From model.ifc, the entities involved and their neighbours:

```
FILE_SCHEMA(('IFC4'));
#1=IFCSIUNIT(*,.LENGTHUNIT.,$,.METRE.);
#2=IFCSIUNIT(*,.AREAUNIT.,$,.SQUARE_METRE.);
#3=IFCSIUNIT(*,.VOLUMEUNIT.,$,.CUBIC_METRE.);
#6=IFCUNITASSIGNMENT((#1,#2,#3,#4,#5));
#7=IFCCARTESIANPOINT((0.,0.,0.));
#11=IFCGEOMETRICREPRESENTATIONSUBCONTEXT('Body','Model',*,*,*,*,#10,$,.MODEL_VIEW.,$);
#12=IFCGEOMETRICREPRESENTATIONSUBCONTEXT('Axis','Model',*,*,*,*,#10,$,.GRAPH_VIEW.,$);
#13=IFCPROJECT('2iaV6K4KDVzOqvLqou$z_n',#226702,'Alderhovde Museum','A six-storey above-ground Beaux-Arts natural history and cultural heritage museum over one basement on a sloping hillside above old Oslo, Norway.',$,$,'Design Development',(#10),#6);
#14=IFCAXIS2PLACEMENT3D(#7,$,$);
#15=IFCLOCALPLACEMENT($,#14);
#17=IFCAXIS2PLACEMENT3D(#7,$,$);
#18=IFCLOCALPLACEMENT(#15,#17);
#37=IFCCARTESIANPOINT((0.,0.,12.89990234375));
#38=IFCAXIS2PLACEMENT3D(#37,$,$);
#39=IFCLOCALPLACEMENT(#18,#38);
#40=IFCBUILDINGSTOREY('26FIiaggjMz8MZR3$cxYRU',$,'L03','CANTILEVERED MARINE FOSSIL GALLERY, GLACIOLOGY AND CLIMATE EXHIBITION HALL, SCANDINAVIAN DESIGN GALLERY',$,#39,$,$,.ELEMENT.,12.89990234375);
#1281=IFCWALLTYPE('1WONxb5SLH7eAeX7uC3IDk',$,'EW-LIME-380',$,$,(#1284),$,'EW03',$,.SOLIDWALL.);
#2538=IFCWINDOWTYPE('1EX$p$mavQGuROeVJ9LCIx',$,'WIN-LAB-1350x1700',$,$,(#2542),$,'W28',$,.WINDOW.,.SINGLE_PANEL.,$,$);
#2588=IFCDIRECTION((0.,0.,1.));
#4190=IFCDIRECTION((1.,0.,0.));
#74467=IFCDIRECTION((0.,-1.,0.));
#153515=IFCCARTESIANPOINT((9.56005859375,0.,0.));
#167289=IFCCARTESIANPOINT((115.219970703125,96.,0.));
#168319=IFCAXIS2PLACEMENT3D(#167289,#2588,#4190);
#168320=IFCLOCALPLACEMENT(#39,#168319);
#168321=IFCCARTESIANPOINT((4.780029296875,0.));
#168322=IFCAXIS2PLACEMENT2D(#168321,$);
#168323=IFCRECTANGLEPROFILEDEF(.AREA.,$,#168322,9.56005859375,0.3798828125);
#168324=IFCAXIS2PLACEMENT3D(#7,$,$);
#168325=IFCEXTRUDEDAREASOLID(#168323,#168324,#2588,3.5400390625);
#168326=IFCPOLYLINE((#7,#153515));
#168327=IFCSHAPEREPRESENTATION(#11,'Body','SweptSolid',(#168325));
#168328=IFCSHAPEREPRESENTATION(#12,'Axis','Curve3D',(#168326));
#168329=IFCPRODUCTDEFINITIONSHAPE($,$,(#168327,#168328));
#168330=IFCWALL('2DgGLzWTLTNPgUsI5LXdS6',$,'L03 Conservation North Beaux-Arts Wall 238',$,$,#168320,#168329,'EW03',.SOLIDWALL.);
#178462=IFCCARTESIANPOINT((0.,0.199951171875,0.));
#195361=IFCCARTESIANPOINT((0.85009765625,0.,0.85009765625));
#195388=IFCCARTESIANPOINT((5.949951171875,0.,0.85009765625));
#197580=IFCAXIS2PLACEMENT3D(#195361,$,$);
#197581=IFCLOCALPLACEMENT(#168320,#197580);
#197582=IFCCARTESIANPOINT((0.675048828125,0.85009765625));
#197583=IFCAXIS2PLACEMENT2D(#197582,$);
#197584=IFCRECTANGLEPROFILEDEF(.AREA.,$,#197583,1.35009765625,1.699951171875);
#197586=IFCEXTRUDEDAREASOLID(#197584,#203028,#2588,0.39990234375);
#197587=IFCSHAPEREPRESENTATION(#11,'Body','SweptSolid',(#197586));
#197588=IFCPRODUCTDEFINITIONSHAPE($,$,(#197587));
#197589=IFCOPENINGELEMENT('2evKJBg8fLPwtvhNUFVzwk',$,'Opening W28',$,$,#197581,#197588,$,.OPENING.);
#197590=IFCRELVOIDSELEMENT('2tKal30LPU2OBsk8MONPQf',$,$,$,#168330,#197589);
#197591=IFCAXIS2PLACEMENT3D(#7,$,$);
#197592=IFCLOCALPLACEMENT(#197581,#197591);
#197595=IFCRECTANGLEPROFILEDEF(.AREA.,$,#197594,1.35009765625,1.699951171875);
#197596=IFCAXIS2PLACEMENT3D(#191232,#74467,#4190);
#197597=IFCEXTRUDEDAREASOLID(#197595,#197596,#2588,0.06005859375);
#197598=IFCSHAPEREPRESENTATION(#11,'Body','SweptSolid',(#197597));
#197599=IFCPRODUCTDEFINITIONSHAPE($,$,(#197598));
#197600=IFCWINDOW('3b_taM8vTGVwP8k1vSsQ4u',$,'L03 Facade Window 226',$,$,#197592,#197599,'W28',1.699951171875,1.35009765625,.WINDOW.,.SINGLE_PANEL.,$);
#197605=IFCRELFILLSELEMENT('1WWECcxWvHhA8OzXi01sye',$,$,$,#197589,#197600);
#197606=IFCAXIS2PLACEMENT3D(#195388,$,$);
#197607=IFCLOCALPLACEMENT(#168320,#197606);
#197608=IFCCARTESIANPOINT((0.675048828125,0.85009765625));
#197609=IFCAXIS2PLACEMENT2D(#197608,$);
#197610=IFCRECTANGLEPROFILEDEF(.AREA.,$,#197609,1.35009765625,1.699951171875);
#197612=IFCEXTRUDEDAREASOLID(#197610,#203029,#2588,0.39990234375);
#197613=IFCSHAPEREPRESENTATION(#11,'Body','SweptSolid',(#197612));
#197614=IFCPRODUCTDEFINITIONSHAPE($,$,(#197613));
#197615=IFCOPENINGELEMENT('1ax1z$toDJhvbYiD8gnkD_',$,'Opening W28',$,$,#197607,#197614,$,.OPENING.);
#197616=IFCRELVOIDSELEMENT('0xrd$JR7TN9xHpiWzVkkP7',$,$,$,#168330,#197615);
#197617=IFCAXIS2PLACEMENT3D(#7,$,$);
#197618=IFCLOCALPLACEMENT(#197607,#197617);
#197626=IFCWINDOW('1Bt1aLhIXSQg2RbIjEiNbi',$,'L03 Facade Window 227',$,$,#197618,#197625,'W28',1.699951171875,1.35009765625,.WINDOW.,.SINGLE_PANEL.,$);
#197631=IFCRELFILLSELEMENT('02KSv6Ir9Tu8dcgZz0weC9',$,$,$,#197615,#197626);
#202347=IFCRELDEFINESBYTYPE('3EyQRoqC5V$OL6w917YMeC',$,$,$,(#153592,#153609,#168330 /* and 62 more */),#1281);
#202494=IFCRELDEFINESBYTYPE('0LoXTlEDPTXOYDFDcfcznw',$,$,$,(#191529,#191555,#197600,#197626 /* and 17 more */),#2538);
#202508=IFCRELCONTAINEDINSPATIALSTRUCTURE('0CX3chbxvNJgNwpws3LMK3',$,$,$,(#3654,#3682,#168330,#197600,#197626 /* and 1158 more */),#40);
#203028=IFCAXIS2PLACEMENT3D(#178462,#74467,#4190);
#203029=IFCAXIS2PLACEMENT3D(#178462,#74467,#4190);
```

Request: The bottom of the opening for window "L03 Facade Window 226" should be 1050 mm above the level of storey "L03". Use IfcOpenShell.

```python
import numpy as np
import ifcopenshell
import ifcopenshell.api.geometry
import ifcopenshell.geom
import ifcopenshell.util.element
import ifcopenshell.util.placement
import ifcopenshell.util.shape
import ifcopenshell.util.unit

model = ifcopenshell.open("model.ifc")
unit_scale = ifcopenshell.util.unit.calculate_unit_scale(model)

window = model.by_guid("3b_taM8vTGVwP8k1vSsQ4u")
opening = window.FillsVoids[0].RelatingOpeningElement
storey = ifcopenshell.util.element.get_container(window, ifc_class="IfcBuildingStorey")
level = ifcopenshell.util.placement.get_local_placement(storey.ObjectPlacement)[2, 3]

# The opening's origin need not be at the sill, so measure its lowest point.
shape = ifcopenshell.geom.create_shape(ifcopenshell.geom.settings(), opening)
bottom = ifcopenshell.util.shape.get_shape_bottom_elevation(shape, shape.geometry) / unit_scale
dz = level + 1.05 / unit_scale - bottom

shift = np.array([0.0, 0.0, dz])
# The window is placed relative to its opening, so it follows when the opening moves.
matrix = ifcopenshell.util.placement.get_local_placement(opening.ObjectPlacement)
matrix[:3, 3] += shift
ifcopenshell.api.geometry.edit_object_placement(
    model, product=opening, matrix=matrix, is_si=False, should_transform_children=True
)

print(f"moved by {dz * unit_scale:+.3f} m")

model.write("model_edited.ifc")
```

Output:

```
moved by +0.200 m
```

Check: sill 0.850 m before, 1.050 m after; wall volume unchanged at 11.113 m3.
